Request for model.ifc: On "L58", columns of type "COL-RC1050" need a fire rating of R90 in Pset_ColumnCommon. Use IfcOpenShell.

First a look at what the model holds.

```python
import ifcopenshell
import ifcopenshell.util.element

model = ifcopenshell.open("model.ifc")
print(model.schema)
storey = next(s for s in model.by_type("IfcBuildingStorey") if s.Name == "L58")
columns = [e for e in ifcopenshell.util.element.get_decomposition(storey) if e.is_a("IfcColumn")]
seen = {}
for e in columns:
    element_type = ifcopenshell.util.element.get_type(e)
    key = (element_type.Name if element_type != e and element_type else None, ifcopenshell.util.element.get_pset(e, "Pset_ColumnCommon", "FireRating"))
    seen[key] = seen.get(key, 0) + 1
for (name, value), count in sorted(seen.items(), key=str):
    print(count, "x", name, "|", value)
```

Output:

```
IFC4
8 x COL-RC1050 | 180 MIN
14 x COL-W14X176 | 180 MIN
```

```python
import ifcopenshell
import ifcopenshell.api.pset
import ifcopenshell.util.element

model = ifcopenshell.open("model.ifc")

storey = next(s for s in model.by_type("IfcBuildingStorey") if s.Name == "L58")
columns = [e for e in ifcopenshell.util.element.get_decomposition(storey) if e.is_a("IfcColumn")]

count = 0
for e in columns:
    element_type = ifcopenshell.util.element.get_type(e)
    if element_type in (None, e) or element_type.Name != "COL-RC1050":
        continue
    found = ifcopenshell.util.element.get_pset(e, "Pset_ColumnCommon", should_inherit=False)
    if found:
        pset = model.by_id(found["id"])
        if len(ifcopenshell.util.element.get_elements_by_pset(pset)) > 1:
            pset = ifcopenshell.api.pset.unshare_pset(model, products=[e], pset=pset)[0]
    else:
        pset = ifcopenshell.api.pset.add_pset(model, product=e, name="Pset_ColumnCommon")
    ifcopenshell.api.pset.edit_pset(model, pset=pset, properties={"FireRating": "R90"})
    count += 1

print(count, "columns updated")

model.write("model-out.ifc")
```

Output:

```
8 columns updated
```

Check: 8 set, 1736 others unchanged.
